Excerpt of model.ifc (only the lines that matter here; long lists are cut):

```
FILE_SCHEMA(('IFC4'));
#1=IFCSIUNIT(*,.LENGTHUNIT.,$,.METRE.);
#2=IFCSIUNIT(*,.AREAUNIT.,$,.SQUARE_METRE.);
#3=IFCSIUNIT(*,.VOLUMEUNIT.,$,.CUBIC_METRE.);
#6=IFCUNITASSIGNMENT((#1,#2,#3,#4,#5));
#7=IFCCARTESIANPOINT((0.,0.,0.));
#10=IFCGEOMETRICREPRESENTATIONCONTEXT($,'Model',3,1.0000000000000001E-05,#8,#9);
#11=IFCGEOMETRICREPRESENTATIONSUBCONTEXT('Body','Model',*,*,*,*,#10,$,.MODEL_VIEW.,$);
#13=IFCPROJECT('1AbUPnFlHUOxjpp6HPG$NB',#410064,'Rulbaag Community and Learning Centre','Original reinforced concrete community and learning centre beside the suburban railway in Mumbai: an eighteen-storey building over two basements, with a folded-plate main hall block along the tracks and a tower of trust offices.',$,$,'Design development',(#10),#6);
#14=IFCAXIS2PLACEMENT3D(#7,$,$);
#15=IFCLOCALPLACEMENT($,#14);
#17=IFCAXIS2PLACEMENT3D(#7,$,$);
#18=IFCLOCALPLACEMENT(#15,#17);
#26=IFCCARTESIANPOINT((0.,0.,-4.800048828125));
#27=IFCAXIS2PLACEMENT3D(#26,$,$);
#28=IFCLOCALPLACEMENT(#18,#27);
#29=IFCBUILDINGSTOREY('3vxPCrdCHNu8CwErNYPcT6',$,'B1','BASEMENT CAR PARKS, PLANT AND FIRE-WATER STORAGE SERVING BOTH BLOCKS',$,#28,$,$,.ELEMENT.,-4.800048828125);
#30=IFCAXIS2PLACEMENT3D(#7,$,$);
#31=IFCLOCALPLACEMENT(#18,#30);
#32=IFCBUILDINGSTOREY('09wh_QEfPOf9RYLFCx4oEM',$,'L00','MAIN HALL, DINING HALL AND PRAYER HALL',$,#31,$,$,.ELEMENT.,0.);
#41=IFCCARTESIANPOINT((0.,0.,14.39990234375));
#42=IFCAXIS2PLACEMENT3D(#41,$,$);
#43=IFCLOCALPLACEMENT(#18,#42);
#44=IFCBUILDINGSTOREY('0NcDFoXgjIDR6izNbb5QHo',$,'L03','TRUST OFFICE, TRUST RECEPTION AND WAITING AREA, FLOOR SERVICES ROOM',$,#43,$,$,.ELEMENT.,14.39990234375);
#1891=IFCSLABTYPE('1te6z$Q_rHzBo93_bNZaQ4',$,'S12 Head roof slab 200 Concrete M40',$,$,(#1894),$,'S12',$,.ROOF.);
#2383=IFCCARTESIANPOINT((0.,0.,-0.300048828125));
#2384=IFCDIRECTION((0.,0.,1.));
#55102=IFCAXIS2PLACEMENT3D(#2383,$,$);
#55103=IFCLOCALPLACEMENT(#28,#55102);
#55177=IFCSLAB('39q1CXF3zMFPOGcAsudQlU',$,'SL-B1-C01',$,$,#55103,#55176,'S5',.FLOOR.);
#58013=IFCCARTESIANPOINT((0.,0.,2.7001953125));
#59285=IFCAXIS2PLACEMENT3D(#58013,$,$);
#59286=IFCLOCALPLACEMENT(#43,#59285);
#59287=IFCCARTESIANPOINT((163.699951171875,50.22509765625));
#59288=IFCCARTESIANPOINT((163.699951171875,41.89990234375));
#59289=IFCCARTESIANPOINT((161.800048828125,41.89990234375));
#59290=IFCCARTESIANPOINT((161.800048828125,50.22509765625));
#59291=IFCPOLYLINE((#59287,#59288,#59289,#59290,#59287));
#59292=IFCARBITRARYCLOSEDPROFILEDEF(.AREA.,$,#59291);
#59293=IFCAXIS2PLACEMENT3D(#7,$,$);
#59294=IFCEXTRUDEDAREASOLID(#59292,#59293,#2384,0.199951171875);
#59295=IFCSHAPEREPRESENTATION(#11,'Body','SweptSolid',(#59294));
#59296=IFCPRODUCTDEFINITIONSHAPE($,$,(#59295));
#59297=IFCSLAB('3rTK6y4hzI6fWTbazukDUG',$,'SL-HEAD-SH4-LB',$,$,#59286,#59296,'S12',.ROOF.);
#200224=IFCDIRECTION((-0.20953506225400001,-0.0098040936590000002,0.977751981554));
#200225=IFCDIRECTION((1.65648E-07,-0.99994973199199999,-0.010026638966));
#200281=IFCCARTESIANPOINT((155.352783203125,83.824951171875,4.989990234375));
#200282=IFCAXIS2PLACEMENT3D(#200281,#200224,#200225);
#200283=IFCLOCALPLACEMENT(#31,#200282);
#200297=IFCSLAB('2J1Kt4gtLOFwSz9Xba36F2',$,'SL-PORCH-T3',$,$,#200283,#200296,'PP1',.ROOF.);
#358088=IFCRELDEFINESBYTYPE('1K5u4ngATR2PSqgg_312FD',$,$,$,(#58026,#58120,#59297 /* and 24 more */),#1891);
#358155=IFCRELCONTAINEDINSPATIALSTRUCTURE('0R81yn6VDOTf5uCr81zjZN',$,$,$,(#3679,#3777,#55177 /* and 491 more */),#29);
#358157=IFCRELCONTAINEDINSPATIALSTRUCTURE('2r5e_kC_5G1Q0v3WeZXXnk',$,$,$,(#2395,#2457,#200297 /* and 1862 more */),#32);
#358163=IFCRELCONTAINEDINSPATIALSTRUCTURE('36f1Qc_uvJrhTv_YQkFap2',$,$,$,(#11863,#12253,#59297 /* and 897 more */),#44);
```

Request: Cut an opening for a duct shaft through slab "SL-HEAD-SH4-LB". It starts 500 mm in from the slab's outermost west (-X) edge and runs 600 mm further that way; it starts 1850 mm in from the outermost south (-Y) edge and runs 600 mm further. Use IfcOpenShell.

```python
import numpy as np
import ifcopenshell
import ifcopenshell.api.feature
import ifcopenshell.api.geometry
import ifcopenshell.api.root
import ifcopenshell.geom
import ifcopenshell.util.placement
import ifcopenshell.util.representation
import ifcopenshell.util.shape
import ifcopenshell.util.unit

model = ifcopenshell.open("model.ifc")
unit_scale = ifcopenshell.util.unit.calculate_unit_scale(model)
settings = ifcopenshell.geom.settings()


def volume(element):
    """Net volume in cubic metres, openings subtracted."""
    shape = ifcopenshell.geom.create_shape(settings, element)
    return ifcopenshell.util.shape.get_volume(shape.geometry)


slab = model.by_guid("3rTK6y4hzI6fWTbazukDUG")
before = volume(slab)

# Extent in the slab's own axes, in metres. The edges named are its -X and -Y sides.
slab_shape = ifcopenshell.geom.create_shape(settings, slab)
vertices = ifcopenshell.util.shape.get_vertices(slab_shape.geometry)
x_min, y_min, bottom = vertices.min(axis=0)
top = vertices[:, 2].max()

opening = ifcopenshell.api.root.create_entity(model, ifc_class="IfcOpeningElement", name="Duct shaft opening", predefined_type="OPENING")
context = ifcopenshell.util.representation.get_context(model, "Model", "Body", "MODEL_VIEW")
width, depth = 0.6, 0.6
outline = [(0.0, 0.0), (width, 0.0), (width, depth), (0.0, depth), (0.0, 0.0)]
# Overshoot both faces by 50 mm so the cut is clean.
shape = ifcopenshell.api.geometry.add_slab_representation(
    model, context=context, depth=top - bottom + 0.1, polyline=outline
)
ifcopenshell.api.geometry.assign_representation(model, product=opening, representation=shape)

matrix = ifcopenshell.util.placement.get_local_placement(slab.ObjectPlacement)
matrix[:, 3] = matrix @ np.append(np.array([x_min + 0.5, y_min + 1.85, bottom - 0.05]) / unit_scale, 1.0)
ifcopenshell.api.geometry.edit_object_placement(model, product=opening, matrix=matrix, is_si=False)
ifcopenshell.api.feature.add_feature(model, feature=opening, element=slab)

after = volume(slab)

print(f"slab volume {before:.3f} -> {after:.3f} m3")

model.write("model_v2.ifc")
```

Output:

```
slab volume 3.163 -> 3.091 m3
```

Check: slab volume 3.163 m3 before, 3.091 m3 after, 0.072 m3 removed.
